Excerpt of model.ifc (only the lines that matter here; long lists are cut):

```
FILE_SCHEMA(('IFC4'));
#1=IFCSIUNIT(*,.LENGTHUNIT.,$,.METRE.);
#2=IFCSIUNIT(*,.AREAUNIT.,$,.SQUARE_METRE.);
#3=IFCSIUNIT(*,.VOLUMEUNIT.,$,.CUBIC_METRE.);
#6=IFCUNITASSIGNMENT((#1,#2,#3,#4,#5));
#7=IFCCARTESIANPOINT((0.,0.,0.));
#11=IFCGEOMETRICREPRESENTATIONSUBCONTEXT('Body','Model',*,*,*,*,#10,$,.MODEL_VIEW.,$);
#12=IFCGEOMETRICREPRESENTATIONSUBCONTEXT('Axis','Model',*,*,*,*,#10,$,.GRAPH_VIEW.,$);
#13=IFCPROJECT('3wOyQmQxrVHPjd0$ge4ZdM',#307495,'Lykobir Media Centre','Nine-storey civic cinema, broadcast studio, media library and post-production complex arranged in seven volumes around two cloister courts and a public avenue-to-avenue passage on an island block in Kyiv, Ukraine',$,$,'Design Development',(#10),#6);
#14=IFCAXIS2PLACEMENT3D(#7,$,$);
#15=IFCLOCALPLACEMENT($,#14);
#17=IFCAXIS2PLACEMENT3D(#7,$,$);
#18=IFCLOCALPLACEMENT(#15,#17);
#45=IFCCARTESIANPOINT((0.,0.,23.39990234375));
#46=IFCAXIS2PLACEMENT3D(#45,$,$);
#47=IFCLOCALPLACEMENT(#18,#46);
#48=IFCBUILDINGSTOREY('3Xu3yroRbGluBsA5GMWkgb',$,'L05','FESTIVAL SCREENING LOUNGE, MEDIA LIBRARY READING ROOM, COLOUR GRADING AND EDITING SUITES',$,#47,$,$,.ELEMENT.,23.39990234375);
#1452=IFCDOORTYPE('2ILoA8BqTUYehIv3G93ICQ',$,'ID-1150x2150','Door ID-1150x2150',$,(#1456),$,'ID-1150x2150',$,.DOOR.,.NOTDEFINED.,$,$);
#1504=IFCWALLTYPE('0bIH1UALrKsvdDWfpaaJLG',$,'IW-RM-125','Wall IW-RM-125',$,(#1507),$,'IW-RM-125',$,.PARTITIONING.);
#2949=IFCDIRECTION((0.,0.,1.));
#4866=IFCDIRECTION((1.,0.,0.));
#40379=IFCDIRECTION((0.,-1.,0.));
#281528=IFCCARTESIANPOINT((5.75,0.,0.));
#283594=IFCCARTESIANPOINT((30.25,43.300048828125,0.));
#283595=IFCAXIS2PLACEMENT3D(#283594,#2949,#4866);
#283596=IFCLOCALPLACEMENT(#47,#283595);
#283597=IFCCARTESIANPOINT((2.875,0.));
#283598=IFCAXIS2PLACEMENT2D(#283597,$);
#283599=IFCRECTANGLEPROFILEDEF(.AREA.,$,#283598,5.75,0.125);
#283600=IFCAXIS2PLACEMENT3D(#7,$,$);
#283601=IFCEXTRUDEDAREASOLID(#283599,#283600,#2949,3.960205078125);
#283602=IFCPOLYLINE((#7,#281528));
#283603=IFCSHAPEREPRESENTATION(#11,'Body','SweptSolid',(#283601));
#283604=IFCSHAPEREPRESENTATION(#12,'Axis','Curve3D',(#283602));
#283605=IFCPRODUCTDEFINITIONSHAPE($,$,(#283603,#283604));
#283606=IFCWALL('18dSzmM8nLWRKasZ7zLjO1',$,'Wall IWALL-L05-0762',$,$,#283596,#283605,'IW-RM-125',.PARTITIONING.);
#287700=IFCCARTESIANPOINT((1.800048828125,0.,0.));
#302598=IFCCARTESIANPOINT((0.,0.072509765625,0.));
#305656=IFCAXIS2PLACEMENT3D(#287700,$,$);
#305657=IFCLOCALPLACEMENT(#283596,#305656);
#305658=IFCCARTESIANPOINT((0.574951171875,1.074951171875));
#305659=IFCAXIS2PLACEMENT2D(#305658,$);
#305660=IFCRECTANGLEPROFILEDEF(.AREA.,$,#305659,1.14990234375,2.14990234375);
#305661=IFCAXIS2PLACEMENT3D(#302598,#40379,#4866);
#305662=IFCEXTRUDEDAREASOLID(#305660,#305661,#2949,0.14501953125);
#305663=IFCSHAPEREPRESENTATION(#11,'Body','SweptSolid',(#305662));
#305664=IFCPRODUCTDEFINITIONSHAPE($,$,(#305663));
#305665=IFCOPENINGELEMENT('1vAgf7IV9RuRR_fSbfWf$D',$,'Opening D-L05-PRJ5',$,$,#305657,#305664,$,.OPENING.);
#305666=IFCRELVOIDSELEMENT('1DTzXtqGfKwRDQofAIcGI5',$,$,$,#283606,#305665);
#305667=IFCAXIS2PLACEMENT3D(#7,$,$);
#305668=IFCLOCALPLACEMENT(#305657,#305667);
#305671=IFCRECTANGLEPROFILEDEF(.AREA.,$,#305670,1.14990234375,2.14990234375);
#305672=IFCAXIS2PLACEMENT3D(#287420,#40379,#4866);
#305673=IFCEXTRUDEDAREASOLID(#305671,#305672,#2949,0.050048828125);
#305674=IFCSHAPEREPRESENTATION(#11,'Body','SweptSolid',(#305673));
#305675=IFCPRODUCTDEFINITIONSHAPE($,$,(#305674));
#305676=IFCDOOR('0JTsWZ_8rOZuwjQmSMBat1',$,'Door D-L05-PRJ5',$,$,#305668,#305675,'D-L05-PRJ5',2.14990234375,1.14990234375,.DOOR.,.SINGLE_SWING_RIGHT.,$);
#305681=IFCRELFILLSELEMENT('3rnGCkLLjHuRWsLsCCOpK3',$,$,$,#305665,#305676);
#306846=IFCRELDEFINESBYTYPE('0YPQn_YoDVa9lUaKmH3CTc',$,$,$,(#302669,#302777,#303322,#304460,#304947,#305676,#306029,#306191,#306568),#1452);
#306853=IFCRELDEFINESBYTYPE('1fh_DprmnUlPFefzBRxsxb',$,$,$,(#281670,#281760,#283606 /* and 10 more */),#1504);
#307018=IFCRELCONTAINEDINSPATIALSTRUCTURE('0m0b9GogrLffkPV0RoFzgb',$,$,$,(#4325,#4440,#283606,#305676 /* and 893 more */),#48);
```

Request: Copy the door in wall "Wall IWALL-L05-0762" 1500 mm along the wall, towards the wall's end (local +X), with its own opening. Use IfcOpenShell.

```python
import ifcopenshell
import ifcopenshell.api.feature
import ifcopenshell.api.geometry
import ifcopenshell.api.root
import ifcopenshell.geom
import ifcopenshell.util.element
import ifcopenshell.util.placement
import ifcopenshell.util.shape
import ifcopenshell.util.unit

model = ifcopenshell.open("model.ifc")
unit_scale = ifcopenshell.util.unit.calculate_unit_scale(model)
settings = ifcopenshell.geom.settings()


def volume(element):
    """Net volume in cubic metres, openings subtracted."""
    shape = ifcopenshell.geom.create_shape(settings, element)
    return ifcopenshell.util.shape.get_volume(shape.geometry)


door = model.by_guid("0JTsWZ_8rOZuwjQmSMBat1")
opening = door.FillsVoids[0].RelatingOpeningElement
wall = opening.VoidsElements[0].RelatingBuildingElement
before = volume(wall)
shift = ifcopenshell.util.placement.get_local_placement(wall.ObjectPlacement)[:3, 0] * 1.5 / unit_scale

# copy_class copies the void relationship, type, container and properties, but no geometry.
new_opening = ifcopenshell.api.root.copy_class(model, product=opening)
new_opening.Representation = ifcopenshell.util.element.copy_deep(
    model, opening.Representation, exclude=["IfcGeometricRepresentationContext", "IfcRepresentationMap"]
)
new_door = ifcopenshell.api.root.copy_class(model, product=door)
new_door.Representation = ifcopenshell.util.element.copy_deep(
    model, door.Representation, exclude=["IfcGeometricRepresentationContext", "IfcRepresentationMap"]
)
new_door.Tag = None
ifcopenshell.api.feature.add_filling(model, opening=new_opening, element=new_door)

for old, new in ((opening, new_opening), (door, new_door)):
    matrix = ifcopenshell.util.placement.get_local_placement(old.ObjectPlacement)
    matrix[:3, 3] += shift
    ifcopenshell.api.geometry.edit_object_placement(model, product=new, matrix=matrix, is_si=False)

after = volume(wall)

print(f"wall volume {before:.3f} -> {after:.3f} m3")

model.write("model_updated.ifc")
```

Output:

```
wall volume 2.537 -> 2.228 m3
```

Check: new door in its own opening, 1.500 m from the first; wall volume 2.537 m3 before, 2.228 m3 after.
